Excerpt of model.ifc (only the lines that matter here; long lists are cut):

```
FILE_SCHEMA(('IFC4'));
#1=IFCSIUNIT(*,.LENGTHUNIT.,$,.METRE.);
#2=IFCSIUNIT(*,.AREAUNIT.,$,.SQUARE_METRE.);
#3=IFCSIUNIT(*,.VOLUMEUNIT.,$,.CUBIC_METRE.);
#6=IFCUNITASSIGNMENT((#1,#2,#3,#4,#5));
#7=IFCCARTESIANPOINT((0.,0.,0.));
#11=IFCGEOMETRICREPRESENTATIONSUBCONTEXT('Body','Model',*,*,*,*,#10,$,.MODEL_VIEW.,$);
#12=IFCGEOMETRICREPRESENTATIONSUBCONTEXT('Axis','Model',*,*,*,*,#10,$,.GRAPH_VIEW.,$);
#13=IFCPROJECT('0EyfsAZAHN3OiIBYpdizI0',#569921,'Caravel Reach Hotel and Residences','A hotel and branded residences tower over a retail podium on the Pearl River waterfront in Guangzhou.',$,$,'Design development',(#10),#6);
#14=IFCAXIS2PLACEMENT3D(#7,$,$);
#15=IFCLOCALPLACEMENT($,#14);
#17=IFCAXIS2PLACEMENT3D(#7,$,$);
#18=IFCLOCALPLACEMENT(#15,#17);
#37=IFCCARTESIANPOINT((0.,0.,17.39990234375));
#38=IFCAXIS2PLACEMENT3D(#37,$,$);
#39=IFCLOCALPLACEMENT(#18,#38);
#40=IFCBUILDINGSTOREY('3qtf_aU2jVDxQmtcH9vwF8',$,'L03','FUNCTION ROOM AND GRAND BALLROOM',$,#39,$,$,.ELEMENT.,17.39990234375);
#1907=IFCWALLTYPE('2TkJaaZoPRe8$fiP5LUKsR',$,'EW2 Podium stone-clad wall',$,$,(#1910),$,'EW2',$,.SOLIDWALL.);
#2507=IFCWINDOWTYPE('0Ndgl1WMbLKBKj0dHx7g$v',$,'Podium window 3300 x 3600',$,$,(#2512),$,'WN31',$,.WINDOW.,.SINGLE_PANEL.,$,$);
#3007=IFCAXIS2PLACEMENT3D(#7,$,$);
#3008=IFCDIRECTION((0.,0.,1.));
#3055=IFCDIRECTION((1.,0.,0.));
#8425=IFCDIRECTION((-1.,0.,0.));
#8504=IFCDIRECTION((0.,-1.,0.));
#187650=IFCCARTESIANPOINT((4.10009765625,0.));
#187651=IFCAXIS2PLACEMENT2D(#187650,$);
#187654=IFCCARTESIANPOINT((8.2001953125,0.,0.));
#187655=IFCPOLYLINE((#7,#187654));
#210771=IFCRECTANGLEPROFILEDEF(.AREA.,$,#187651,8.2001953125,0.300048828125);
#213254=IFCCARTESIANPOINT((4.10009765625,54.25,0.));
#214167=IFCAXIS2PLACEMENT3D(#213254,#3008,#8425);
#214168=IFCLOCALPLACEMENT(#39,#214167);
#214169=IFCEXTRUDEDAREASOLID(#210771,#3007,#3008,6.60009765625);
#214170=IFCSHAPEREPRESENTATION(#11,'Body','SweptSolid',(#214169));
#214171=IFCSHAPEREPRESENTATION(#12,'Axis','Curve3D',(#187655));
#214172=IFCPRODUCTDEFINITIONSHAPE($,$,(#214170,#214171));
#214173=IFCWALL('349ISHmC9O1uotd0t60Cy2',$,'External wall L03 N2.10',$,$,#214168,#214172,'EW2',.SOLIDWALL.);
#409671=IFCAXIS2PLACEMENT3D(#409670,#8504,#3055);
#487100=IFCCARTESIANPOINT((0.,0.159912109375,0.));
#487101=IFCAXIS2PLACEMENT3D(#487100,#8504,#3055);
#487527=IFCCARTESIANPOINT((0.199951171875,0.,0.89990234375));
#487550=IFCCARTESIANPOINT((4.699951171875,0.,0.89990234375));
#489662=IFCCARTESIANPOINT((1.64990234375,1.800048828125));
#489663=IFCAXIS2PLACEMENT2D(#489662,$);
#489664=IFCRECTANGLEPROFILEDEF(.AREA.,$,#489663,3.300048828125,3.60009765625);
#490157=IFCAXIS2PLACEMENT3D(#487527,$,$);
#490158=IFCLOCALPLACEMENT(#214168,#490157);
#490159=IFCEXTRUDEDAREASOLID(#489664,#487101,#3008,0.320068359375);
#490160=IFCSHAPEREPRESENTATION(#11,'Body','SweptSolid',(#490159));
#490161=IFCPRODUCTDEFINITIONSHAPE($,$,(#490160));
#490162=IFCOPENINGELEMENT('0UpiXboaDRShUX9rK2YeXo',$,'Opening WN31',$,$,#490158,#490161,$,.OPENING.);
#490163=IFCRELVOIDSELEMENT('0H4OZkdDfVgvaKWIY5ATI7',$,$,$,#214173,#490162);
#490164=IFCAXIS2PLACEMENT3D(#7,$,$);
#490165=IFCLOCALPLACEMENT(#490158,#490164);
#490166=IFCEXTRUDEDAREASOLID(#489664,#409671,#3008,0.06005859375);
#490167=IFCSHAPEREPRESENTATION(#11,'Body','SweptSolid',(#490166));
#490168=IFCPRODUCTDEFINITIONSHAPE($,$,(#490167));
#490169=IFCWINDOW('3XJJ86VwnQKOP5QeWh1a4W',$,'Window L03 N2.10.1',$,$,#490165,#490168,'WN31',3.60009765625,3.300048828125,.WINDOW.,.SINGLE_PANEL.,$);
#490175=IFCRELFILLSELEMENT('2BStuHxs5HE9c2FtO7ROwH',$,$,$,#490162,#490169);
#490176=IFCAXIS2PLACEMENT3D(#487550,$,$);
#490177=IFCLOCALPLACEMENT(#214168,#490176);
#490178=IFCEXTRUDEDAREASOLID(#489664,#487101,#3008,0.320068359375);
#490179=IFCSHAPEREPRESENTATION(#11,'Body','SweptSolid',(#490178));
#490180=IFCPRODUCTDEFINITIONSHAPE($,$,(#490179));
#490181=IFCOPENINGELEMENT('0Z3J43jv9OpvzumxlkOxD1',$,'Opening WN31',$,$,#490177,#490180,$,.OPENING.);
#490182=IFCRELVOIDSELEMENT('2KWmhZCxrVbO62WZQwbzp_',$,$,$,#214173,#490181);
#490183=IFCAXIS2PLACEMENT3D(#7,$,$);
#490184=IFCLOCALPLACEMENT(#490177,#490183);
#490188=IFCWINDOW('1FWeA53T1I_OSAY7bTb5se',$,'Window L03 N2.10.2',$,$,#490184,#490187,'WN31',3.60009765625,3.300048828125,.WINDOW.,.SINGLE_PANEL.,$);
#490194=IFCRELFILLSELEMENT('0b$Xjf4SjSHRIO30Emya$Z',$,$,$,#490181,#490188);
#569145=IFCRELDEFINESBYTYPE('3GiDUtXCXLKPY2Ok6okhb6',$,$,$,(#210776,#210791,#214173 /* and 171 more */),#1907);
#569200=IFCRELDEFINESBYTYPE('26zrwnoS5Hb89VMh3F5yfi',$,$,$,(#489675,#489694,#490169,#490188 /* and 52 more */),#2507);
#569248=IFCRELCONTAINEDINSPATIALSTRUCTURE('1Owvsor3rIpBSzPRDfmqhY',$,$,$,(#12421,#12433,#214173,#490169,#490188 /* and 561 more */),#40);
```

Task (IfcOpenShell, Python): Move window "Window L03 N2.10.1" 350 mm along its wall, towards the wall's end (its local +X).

```python
import ifcopenshell
import ifcopenshell.api.geometry
import ifcopenshell.util.placement

model = ifcopenshell.open("model.ifc")

window = model.by_guid("3XJJ86VwnQKOP5QeWh1a4W")
opening = window.FillsVoids[0].RelatingOpeningElement
wall = opening.VoidsElements[0].RelatingBuildingElement

wall_matrix = ifcopenshell.util.placement.get_local_placement(wall.ObjectPlacement)
shift = wall_matrix[:3, 0] * 0.35
before = ifcopenshell.util.placement.get_local_placement(window.ObjectPlacement)[:3, 3].copy()

# The window is placed relative to its opening, so it follows when the opening moves.
matrix = ifcopenshell.util.placement.get_local_placement(opening.ObjectPlacement)
matrix[:3, 3] += shift
ifcopenshell.api.geometry.edit_object_placement(
    model, product=opening, matrix=matrix, is_si=False, should_transform_children=True
)

after = ifcopenshell.util.placement.get_local_placement(window.ObjectPlacement)[:3, 3]
print("window moved by", (after - before).round(3) + 0.0)

model.write("model-out.ifc")
```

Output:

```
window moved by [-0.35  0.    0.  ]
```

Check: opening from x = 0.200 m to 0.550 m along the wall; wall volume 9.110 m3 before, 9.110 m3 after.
